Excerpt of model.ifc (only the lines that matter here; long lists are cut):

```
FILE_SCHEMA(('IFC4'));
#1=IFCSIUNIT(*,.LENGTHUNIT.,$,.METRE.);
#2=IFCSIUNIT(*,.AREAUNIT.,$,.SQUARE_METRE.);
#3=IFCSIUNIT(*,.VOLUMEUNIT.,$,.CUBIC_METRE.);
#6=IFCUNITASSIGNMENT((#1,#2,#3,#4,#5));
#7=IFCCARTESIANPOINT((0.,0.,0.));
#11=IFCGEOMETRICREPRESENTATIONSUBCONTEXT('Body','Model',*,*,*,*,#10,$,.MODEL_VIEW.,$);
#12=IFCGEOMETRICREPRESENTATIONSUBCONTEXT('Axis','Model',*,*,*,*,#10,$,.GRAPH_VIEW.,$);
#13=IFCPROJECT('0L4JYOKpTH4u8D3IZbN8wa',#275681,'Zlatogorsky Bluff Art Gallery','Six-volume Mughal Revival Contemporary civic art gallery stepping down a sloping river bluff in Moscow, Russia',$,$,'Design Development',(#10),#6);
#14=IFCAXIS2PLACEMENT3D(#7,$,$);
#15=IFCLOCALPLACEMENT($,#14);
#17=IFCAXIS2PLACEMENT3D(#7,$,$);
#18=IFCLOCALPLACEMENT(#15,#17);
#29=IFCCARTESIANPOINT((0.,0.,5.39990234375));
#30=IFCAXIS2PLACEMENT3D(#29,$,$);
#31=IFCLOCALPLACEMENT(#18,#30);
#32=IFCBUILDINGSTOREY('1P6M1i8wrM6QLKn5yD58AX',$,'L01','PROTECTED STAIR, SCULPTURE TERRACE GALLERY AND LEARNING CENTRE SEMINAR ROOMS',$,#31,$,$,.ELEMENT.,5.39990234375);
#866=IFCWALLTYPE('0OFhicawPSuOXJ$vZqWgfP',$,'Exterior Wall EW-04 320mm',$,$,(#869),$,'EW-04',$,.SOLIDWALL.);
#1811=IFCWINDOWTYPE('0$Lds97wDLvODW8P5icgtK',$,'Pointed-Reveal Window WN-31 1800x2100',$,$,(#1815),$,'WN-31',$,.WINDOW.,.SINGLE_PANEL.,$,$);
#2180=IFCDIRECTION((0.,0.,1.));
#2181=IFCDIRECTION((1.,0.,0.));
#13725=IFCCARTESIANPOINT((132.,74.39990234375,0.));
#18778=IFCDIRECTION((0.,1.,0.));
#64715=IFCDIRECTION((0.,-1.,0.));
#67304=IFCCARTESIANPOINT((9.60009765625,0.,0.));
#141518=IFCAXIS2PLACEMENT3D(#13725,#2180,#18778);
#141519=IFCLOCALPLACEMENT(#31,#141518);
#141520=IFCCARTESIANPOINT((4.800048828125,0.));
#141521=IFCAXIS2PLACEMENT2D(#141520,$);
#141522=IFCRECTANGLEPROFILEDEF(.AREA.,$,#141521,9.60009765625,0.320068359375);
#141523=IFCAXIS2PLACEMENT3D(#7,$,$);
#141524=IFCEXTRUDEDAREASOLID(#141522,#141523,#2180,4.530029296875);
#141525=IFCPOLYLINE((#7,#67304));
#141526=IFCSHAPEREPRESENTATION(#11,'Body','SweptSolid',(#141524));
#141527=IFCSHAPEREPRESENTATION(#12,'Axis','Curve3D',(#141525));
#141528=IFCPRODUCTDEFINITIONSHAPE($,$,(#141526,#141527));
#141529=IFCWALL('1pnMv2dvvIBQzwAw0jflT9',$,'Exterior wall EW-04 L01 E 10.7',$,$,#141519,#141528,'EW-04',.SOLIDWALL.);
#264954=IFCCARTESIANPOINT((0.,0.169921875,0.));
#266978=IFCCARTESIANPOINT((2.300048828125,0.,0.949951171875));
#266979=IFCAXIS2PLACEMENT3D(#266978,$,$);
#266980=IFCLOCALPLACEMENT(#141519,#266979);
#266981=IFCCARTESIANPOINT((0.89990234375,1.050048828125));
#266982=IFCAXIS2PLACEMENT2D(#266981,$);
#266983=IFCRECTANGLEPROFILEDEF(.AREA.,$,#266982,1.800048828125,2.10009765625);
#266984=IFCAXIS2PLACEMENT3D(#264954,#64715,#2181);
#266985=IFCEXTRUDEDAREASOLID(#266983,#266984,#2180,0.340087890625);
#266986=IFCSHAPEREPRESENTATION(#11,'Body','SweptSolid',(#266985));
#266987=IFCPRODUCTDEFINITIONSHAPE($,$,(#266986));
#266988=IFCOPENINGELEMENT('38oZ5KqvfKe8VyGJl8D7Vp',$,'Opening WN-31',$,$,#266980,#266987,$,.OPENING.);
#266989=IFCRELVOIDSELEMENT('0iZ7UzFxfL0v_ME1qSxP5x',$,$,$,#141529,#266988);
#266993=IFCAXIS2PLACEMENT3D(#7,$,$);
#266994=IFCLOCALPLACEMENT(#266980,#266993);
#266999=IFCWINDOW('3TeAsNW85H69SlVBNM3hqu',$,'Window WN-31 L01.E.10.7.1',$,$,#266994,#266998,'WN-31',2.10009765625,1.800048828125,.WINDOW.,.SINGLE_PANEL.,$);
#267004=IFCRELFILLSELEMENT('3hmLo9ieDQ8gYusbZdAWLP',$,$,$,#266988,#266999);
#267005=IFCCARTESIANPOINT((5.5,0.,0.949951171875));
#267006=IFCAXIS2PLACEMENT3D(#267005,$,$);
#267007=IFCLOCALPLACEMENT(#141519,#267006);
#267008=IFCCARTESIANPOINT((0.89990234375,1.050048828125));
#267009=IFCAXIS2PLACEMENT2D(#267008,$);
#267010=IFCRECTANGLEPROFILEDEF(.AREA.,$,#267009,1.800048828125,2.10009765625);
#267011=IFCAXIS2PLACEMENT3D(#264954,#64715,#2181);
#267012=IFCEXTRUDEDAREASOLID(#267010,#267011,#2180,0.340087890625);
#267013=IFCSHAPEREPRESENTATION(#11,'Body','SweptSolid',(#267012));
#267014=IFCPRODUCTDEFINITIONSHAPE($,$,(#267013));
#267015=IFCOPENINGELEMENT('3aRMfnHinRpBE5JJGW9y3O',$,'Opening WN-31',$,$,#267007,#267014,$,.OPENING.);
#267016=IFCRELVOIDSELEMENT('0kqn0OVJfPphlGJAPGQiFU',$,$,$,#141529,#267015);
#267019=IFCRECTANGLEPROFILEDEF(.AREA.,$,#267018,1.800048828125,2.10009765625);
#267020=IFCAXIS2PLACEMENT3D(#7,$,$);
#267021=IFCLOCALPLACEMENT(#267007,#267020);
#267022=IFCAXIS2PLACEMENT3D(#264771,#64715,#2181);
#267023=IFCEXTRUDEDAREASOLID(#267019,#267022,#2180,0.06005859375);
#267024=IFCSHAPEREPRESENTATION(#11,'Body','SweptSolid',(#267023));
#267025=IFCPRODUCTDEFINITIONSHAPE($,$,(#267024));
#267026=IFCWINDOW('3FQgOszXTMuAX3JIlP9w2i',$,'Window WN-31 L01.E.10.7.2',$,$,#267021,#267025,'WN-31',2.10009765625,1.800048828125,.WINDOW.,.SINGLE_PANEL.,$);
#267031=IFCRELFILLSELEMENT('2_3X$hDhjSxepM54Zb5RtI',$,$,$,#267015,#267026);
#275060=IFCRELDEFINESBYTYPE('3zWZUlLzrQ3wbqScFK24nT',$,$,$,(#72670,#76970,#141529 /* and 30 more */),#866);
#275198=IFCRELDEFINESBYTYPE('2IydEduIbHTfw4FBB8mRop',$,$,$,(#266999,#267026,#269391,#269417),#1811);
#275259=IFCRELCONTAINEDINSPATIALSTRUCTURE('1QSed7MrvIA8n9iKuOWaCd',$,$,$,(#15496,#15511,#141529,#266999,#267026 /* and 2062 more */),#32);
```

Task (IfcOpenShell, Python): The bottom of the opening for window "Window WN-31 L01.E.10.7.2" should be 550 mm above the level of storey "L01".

```python
import numpy as np
import ifcopenshell
import ifcopenshell.api.geometry
import ifcopenshell.geom
import ifcopenshell.util.element
import ifcopenshell.util.placement
import ifcopenshell.util.shape
import ifcopenshell.util.unit

model = ifcopenshell.open("model.ifc")
unit_scale = ifcopenshell.util.unit.calculate_unit_scale(model)

window = model.by_guid("3FQgOszXTMuAX3JIlP9w2i")
opening = window.FillsVoids[0].RelatingOpeningElement
storey = ifcopenshell.util.element.get_container(window, ifc_class="IfcBuildingStorey")
level = ifcopenshell.util.placement.get_local_placement(storey.ObjectPlacement)[2, 3]

# The opening's origin need not be at the sill, so measure its lowest point.
shape = ifcopenshell.geom.create_shape(ifcopenshell.geom.settings(), opening)
bottom = ifcopenshell.util.shape.get_shape_bottom_elevation(shape, shape.geometry) / unit_scale
dz = level + 0.55 - bottom

shift = np.array([0.0, 0.0, dz])
# The window is placed relative to its opening, so it follows when the opening moves.
matrix = ifcopenshell.util.placement.get_local_placement(opening.ObjectPlacement)
matrix[:3, 3] += shift
ifcopenshell.api.geometry.edit_object_placement(
    model, product=opening, matrix=matrix, is_si=False, should_transform_children=True
)

print(f"moved by {dz * unit_scale:+.3f} m")

model.write("model_v2.ifc")
```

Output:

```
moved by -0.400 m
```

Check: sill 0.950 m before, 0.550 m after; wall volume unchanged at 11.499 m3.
